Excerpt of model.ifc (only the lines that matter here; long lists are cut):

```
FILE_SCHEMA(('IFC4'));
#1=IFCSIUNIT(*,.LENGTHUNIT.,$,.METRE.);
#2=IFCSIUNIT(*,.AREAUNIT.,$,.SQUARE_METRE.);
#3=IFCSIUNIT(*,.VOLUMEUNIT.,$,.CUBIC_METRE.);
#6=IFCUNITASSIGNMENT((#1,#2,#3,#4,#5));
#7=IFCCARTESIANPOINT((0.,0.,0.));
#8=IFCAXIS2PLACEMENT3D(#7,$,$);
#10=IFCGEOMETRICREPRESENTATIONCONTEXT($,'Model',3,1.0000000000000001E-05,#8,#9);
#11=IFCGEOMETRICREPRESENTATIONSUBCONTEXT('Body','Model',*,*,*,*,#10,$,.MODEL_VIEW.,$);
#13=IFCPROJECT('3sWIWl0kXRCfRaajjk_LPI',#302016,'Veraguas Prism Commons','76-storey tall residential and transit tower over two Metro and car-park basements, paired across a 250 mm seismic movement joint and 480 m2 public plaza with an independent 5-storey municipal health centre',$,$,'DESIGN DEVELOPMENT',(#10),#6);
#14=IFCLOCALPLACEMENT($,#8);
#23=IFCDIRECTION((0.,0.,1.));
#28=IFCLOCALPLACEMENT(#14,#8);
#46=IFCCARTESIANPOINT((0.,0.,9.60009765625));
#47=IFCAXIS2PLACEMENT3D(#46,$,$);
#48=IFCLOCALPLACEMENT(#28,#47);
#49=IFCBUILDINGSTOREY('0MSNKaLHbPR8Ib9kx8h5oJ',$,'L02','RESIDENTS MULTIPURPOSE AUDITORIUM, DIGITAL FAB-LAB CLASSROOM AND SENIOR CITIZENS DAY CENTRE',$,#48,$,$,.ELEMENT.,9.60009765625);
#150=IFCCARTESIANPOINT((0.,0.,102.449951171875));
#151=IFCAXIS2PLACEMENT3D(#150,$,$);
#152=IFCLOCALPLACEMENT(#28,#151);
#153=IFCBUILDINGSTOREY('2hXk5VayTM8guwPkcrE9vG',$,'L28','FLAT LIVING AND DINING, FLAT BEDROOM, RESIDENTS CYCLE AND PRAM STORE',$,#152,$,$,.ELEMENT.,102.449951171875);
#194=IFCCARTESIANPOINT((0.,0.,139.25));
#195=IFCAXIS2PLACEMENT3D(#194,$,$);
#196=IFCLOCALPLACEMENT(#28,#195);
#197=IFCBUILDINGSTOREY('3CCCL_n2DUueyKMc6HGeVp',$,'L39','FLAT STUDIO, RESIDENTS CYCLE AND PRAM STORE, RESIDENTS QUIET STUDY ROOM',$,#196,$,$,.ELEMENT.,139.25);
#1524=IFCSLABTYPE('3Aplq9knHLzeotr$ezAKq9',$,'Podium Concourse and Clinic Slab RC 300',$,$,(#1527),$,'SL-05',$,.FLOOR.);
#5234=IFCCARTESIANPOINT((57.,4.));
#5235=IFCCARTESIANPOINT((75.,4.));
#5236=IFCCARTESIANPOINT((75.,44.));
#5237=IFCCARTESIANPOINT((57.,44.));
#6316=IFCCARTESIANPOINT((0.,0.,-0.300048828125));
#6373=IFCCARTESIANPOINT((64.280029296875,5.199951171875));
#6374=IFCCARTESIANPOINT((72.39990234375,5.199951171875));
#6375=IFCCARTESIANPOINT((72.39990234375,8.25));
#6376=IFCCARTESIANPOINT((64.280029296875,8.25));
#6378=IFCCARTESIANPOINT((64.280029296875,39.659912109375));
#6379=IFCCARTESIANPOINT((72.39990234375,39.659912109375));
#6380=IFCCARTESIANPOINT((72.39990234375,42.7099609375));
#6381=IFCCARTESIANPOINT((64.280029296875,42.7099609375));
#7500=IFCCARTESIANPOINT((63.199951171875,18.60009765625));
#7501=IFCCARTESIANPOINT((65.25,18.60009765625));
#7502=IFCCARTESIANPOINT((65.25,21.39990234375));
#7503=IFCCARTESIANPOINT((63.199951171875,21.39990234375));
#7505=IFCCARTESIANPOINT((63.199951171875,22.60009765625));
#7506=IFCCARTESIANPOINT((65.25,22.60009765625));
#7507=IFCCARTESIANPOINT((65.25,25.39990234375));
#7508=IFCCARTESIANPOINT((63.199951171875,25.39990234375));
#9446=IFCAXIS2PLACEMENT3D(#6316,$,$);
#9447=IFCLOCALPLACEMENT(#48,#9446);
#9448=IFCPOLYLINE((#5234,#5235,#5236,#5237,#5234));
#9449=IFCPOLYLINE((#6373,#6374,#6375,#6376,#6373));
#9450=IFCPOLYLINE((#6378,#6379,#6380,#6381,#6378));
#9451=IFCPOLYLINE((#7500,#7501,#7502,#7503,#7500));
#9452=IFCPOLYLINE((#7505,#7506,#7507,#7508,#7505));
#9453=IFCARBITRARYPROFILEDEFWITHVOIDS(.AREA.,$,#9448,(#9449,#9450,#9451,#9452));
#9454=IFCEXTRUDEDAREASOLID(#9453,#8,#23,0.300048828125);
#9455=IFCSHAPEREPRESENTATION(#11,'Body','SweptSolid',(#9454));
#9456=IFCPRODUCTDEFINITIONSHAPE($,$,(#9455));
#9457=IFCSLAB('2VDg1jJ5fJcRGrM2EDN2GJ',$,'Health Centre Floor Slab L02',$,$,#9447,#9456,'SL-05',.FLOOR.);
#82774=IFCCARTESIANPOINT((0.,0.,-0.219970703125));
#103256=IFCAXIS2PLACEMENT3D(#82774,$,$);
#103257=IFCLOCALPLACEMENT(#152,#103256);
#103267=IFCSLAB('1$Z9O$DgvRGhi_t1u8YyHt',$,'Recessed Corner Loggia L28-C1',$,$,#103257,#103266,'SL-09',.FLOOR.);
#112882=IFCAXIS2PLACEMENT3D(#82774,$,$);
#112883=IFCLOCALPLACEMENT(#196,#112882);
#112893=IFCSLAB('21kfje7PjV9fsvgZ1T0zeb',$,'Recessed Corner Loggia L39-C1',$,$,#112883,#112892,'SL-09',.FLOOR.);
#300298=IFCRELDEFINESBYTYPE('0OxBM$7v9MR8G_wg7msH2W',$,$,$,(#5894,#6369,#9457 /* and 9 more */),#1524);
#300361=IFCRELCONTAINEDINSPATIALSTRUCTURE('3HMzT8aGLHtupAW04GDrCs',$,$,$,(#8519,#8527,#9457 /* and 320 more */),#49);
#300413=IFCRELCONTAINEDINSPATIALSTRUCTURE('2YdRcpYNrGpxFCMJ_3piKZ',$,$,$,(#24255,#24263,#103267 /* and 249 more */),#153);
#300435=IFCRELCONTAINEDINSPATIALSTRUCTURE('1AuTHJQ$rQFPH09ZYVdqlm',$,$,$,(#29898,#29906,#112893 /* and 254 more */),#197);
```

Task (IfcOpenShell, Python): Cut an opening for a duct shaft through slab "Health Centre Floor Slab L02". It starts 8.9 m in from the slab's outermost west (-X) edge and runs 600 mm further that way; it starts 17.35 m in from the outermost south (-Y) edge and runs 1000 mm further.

```python
import numpy as np
import ifcopenshell
import ifcopenshell.api.feature
import ifcopenshell.api.geometry
import ifcopenshell.api.root
import ifcopenshell.geom
import ifcopenshell.util.placement
import ifcopenshell.util.representation
import ifcopenshell.util.shape
import ifcopenshell.util.unit

model = ifcopenshell.open("model.ifc")
unit_scale = ifcopenshell.util.unit.calculate_unit_scale(model)
settings = ifcopenshell.geom.settings()


def volume(element):
    """Net volume in cubic metres, openings subtracted."""
    shape = ifcopenshell.geom.create_shape(settings, element)
    return ifcopenshell.util.shape.get_volume(shape.geometry)


slab = model.by_id(9457)
before = volume(slab)

# Extent in the slab's own axes, in metres. The edges named are its -X and -Y sides.
slab_shape = ifcopenshell.geom.create_shape(settings, slab)
vertices = ifcopenshell.util.shape.get_vertices(slab_shape.geometry)
x_min, y_min, bottom = vertices.min(axis=0)
top = vertices[:, 2].max()

opening = ifcopenshell.api.root.create_entity(model, ifc_class="IfcOpeningElement", name="Duct shaft opening", predefined_type="OPENING")
context = ifcopenshell.util.representation.get_context(model, "Model", "Body", "MODEL_VIEW")
width, depth = 0.6, 1
outline = [(0.0, 0.0), (width, 0.0), (width, depth), (0.0, depth), (0.0, 0.0)]
# Overshoot both faces by 50 mm so the cut is clean.
shape = ifcopenshell.api.geometry.add_slab_representation(
    model, context=context, depth=top - bottom + 0.1, polyline=outline
)
ifcopenshell.api.geometry.assign_representation(model, product=opening, representation=shape)

matrix = ifcopenshell.util.placement.get_local_placement(slab.ObjectPlacement)
matrix[:, 3] = matrix @ np.append(np.array([x_min + 8.9, y_min + 17.35, bottom - 0.05]) / unit_scale, 1.0)
ifcopenshell.api.geometry.edit_object_placement(model, product=opening, matrix=matrix, is_si=False)
ifcopenshell.api.feature.add_feature(model, feature=opening, element=slab)

after = volume(slab)

print(f"slab volume {before:.3f} -> {after:.3f} m3")

model.write("model_rev.ifc")
```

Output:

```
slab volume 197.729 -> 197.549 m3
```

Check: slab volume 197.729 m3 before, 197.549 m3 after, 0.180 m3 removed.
